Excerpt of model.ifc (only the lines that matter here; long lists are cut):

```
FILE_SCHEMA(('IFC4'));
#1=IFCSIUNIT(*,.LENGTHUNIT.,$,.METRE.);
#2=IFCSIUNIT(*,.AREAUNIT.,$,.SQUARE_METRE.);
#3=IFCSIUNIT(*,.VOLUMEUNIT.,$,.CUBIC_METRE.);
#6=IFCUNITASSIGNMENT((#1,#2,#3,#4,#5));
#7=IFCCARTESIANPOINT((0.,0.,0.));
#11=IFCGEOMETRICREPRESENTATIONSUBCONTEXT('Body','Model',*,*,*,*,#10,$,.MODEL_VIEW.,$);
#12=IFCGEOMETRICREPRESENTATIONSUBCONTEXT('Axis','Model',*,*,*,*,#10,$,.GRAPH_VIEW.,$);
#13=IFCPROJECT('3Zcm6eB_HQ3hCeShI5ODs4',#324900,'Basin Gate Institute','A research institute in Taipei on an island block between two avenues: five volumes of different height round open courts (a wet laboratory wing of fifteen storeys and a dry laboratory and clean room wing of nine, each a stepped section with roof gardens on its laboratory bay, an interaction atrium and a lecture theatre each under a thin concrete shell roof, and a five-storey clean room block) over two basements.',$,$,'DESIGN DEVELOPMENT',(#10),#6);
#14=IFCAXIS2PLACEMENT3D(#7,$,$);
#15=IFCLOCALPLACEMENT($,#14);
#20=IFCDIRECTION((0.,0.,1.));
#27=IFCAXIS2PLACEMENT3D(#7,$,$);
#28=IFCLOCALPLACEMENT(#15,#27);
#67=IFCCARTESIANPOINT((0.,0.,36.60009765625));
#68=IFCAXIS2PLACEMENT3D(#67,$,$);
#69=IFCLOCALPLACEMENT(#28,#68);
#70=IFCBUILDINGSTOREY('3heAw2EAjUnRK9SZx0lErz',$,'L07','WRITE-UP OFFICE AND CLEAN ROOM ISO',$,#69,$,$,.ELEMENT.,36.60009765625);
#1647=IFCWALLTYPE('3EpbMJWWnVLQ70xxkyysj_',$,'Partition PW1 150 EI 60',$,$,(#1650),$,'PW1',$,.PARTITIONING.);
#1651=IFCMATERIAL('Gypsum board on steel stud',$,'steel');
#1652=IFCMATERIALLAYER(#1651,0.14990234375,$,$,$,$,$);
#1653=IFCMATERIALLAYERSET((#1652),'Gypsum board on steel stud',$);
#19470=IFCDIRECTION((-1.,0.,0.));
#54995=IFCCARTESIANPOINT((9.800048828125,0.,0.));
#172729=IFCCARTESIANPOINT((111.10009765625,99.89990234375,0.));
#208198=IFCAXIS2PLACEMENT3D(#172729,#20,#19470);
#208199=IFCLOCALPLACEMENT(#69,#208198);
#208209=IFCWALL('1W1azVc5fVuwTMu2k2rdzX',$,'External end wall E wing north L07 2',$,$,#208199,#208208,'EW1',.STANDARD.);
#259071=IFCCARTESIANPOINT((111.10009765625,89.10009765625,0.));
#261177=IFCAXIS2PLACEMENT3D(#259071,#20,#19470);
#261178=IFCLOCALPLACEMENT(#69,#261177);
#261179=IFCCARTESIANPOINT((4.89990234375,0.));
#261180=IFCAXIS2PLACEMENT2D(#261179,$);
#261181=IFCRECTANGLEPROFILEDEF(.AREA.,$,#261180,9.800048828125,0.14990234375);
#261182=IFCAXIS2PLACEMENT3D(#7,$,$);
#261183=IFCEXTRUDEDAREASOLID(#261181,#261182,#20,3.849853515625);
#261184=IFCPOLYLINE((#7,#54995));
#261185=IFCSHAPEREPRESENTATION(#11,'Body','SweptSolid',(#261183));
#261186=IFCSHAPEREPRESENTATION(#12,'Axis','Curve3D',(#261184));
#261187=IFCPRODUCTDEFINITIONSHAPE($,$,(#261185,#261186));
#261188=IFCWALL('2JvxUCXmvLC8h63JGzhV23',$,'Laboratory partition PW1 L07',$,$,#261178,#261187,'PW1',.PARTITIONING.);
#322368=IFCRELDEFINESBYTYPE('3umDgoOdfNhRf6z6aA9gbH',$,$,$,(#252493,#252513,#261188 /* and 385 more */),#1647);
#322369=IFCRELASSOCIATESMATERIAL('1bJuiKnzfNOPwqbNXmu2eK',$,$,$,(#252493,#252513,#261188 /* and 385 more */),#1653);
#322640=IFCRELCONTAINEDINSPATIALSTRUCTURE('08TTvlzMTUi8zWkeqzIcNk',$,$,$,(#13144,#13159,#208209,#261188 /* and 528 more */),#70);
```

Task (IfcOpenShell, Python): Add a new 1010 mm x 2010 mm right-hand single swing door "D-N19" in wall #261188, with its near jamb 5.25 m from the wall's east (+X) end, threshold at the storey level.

```python
import numpy as np
import ifcopenshell
import ifcopenshell.api.feature
import ifcopenshell.api.geometry
import ifcopenshell.api.root
import ifcopenshell.api.spatial
import ifcopenshell.geom
import ifcopenshell.util.element
import ifcopenshell.util.placement
import ifcopenshell.util.representation
import ifcopenshell.util.shape
import ifcopenshell.util.unit

model = ifcopenshell.open("model.ifc")
unit_scale = ifcopenshell.util.unit.calculate_unit_scale(model)
settings = ifcopenshell.geom.settings()


def volume(element):
    """Net volume in cubic metres, openings subtracted."""
    shape = ifcopenshell.geom.create_shape(settings, element)
    return ifcopenshell.util.shape.get_volume(shape.geometry)


wall = model.by_id(261188)
storey = ifcopenshell.util.element.get_container(wall, ifc_class="IfcBuildingStorey")
context = ifcopenshell.util.representation.get_context(model, "Model", "Body", "MODEL_VIEW")
before = volume(wall)

width, height, from_end, sill = 1.01, 2.01, 5.25, 0.0  # metres

# The wall runs along its own X axis, and the end named is its -X end.
wall_shape = ifcopenshell.geom.create_shape(settings, wall)
x, y, z = ifcopenshell.util.shape.get_vertices(wall_shape.geometry).T
start = x.min() + from_end
face, thickness = float(y.min()), float(y.max() - y.min())
wall_matrix = ifcopenshell.util.placement.get_local_placement(wall.ObjectPlacement)
level = ifcopenshell.util.placement.get_local_placement(storey.ObjectPlacement)[2, 3]


def in_wall(x, y):
    """Placement at x, y metres in the wall's axes, at sill height."""
    matrix = wall_matrix.copy()
    matrix[:, 3] = wall_matrix @ np.array([x / unit_scale, y / unit_scale, 0.0, 1.0])
    matrix[2, 3] = level + sill / unit_scale
    return matrix


# Opening: a box that overshoots both wall faces by 50 mm.
opening = ifcopenshell.api.root.create_entity(model, ifc_class="IfcOpeningElement", predefined_type="OPENING")
box = ifcopenshell.api.geometry.add_wall_representation(
    model, context=context, length=width, height=height, thickness=thickness + 0.1
)
ifcopenshell.api.geometry.assign_representation(model, product=opening, representation=box)
ifcopenshell.api.geometry.edit_object_placement(model, product=opening, matrix=in_wall(start, face - 0.05), is_si=False)
ifcopenshell.api.feature.add_feature(model, feature=opening, element=wall)

door = ifcopenshell.api.root.create_entity(model, ifc_class="IfcDoor", name="D-N19", predefined_type="DOOR")
door.OverallWidth, door.OverallHeight = width / unit_scale, height / unit_scale
door.OperationType = "SINGLE_SWING_RIGHT"
body = ifcopenshell.api.geometry.add_door_representation(
    model,
    context=context,
    overall_width=door.OverallWidth,
    overall_height=door.OverallHeight,
    operation_type="SINGLE_SWING_RIGHT",
    lining_properties={"LiningDepth": thickness / unit_scale, "ThresholdDepth": thickness / unit_scale},
)
ifcopenshell.api.geometry.assign_representation(model, product=door, representation=body)
ifcopenshell.api.spatial.assign_container(model, products=[door], relating_structure=storey)
ifcopenshell.api.feature.add_filling(model, opening=opening, element=door)

# The lining spans the wall, so the door starts at the wall face.
ifcopenshell.api.geometry.edit_object_placement(model, product=door, matrix=in_wall(start, face), is_si=False)

after = volume(wall)

print(f"wall volume {before:.3f} -> {after:.3f} m3")

model.write("model-out.ifc")
```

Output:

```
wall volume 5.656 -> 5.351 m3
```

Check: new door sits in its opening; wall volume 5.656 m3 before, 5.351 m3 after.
